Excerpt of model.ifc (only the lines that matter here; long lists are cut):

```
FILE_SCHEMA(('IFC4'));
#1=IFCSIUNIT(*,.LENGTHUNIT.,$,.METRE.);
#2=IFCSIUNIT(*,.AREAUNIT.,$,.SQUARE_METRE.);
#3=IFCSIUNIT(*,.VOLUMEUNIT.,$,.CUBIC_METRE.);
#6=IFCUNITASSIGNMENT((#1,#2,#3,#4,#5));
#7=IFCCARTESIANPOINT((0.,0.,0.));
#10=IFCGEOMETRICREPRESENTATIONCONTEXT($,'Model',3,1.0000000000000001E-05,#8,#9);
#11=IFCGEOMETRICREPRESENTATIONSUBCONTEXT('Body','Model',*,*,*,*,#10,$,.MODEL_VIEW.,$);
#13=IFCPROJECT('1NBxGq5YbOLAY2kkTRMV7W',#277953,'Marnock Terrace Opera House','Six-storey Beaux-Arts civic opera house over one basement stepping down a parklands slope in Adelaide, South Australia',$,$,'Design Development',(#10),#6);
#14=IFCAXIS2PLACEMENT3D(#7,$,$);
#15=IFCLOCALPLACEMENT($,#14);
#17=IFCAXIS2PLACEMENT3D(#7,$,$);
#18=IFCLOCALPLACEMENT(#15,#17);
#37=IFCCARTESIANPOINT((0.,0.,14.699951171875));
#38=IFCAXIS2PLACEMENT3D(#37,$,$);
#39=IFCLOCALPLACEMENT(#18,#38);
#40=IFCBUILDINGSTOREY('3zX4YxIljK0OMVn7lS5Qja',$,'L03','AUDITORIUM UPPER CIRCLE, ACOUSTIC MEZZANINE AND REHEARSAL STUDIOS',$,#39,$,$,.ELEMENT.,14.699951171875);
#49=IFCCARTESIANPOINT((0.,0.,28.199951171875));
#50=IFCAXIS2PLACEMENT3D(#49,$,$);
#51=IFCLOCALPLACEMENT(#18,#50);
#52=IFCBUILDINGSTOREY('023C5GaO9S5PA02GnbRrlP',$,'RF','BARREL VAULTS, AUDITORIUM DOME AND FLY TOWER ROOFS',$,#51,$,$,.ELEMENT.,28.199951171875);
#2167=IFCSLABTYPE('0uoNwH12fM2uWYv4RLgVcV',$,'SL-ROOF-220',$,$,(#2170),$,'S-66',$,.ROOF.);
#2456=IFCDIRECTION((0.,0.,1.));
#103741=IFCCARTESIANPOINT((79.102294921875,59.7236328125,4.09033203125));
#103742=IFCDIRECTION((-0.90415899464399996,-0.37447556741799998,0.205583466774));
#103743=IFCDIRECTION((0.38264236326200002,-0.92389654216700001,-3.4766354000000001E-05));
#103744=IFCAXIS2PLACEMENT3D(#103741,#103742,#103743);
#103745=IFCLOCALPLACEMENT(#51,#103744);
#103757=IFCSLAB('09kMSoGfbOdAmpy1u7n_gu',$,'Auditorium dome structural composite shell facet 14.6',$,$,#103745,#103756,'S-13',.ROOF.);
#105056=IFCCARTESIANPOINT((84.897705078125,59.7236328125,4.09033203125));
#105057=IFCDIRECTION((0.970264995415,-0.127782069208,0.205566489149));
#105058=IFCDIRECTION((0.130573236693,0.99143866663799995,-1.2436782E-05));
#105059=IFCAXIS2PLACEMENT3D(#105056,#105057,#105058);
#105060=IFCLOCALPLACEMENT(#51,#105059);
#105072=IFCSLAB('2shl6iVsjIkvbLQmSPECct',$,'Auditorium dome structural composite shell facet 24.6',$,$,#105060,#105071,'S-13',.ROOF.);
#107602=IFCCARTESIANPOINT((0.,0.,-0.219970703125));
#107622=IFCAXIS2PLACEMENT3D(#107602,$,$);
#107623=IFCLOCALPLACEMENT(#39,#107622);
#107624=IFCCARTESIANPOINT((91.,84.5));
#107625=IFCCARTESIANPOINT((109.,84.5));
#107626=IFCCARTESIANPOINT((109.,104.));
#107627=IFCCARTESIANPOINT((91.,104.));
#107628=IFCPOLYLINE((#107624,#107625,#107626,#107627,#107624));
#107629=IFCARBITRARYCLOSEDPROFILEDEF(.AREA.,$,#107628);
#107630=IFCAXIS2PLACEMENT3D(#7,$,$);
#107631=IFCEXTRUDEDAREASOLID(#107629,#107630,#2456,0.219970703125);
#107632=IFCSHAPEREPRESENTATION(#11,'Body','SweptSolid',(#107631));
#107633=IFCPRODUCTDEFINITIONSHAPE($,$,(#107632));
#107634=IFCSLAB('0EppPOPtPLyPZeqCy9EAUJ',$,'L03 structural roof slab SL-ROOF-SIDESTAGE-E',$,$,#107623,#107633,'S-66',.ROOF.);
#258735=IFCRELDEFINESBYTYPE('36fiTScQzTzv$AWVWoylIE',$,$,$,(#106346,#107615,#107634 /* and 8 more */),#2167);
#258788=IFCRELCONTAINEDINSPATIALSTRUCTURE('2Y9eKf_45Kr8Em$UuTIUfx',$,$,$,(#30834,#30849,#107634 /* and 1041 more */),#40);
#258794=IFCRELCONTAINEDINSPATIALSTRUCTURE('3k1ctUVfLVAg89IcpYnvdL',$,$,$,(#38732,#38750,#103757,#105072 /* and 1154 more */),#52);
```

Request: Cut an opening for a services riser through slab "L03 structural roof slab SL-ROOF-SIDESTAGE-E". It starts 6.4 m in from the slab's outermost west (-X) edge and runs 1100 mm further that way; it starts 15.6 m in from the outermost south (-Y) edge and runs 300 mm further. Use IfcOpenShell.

```python
import numpy as np
import ifcopenshell
import ifcopenshell.api.feature
import ifcopenshell.api.geometry
import ifcopenshell.api.root
import ifcopenshell.geom
import ifcopenshell.util.placement
import ifcopenshell.util.representation
import ifcopenshell.util.shape
import ifcopenshell.util.unit

model = ifcopenshell.open("model.ifc")
unit_scale = ifcopenshell.util.unit.calculate_unit_scale(model)
settings = ifcopenshell.geom.settings()


def volume(element):
    """Net volume in cubic metres, openings subtracted."""
    shape = ifcopenshell.geom.create_shape(settings, element)
    return ifcopenshell.util.shape.get_volume(shape.geometry)


slab = model.by_id(107634)
before = volume(slab)

# Extent in the slab's own axes, in metres. The edges named are its -X and -Y sides.
slab_shape = ifcopenshell.geom.create_shape(settings, slab)
vertices = ifcopenshell.util.shape.get_vertices(slab_shape.geometry)
x_min, y_min, bottom = vertices.min(axis=0)
top = vertices[:, 2].max()

opening = ifcopenshell.api.root.create_entity(model, ifc_class="IfcOpeningElement", name="Services riser opening", predefined_type="OPENING")
context = ifcopenshell.util.representation.get_context(model, "Model", "Body", "MODEL_VIEW")
width, depth = 1.1, 0.3
outline = [(0.0, 0.0), (width, 0.0), (width, depth), (0.0, depth), (0.0, 0.0)]
# Overshoot both faces by 50 mm so the cut is clean.
shape = ifcopenshell.api.geometry.add_slab_representation(
    model, context=context, depth=top - bottom + 0.1, polyline=outline
)
ifcopenshell.api.geometry.assign_representation(model, product=opening, representation=shape)

matrix = ifcopenshell.util.placement.get_local_placement(slab.ObjectPlacement)
matrix[:, 3] = matrix @ np.append(np.array([x_min + 6.4, y_min + 15.6, bottom - 0.05]) / unit_scale, 1.0)
ifcopenshell.api.geometry.edit_object_placement(model, product=opening, matrix=matrix, is_si=False)
ifcopenshell.api.feature.add_feature(model, feature=opening, element=slab)

after = volume(slab)

print(f"slab volume {before:.3f} -> {after:.3f} m3")

model.write("model_v2.ifc")
```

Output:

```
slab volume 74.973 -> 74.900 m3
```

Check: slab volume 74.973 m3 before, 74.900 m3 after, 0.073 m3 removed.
